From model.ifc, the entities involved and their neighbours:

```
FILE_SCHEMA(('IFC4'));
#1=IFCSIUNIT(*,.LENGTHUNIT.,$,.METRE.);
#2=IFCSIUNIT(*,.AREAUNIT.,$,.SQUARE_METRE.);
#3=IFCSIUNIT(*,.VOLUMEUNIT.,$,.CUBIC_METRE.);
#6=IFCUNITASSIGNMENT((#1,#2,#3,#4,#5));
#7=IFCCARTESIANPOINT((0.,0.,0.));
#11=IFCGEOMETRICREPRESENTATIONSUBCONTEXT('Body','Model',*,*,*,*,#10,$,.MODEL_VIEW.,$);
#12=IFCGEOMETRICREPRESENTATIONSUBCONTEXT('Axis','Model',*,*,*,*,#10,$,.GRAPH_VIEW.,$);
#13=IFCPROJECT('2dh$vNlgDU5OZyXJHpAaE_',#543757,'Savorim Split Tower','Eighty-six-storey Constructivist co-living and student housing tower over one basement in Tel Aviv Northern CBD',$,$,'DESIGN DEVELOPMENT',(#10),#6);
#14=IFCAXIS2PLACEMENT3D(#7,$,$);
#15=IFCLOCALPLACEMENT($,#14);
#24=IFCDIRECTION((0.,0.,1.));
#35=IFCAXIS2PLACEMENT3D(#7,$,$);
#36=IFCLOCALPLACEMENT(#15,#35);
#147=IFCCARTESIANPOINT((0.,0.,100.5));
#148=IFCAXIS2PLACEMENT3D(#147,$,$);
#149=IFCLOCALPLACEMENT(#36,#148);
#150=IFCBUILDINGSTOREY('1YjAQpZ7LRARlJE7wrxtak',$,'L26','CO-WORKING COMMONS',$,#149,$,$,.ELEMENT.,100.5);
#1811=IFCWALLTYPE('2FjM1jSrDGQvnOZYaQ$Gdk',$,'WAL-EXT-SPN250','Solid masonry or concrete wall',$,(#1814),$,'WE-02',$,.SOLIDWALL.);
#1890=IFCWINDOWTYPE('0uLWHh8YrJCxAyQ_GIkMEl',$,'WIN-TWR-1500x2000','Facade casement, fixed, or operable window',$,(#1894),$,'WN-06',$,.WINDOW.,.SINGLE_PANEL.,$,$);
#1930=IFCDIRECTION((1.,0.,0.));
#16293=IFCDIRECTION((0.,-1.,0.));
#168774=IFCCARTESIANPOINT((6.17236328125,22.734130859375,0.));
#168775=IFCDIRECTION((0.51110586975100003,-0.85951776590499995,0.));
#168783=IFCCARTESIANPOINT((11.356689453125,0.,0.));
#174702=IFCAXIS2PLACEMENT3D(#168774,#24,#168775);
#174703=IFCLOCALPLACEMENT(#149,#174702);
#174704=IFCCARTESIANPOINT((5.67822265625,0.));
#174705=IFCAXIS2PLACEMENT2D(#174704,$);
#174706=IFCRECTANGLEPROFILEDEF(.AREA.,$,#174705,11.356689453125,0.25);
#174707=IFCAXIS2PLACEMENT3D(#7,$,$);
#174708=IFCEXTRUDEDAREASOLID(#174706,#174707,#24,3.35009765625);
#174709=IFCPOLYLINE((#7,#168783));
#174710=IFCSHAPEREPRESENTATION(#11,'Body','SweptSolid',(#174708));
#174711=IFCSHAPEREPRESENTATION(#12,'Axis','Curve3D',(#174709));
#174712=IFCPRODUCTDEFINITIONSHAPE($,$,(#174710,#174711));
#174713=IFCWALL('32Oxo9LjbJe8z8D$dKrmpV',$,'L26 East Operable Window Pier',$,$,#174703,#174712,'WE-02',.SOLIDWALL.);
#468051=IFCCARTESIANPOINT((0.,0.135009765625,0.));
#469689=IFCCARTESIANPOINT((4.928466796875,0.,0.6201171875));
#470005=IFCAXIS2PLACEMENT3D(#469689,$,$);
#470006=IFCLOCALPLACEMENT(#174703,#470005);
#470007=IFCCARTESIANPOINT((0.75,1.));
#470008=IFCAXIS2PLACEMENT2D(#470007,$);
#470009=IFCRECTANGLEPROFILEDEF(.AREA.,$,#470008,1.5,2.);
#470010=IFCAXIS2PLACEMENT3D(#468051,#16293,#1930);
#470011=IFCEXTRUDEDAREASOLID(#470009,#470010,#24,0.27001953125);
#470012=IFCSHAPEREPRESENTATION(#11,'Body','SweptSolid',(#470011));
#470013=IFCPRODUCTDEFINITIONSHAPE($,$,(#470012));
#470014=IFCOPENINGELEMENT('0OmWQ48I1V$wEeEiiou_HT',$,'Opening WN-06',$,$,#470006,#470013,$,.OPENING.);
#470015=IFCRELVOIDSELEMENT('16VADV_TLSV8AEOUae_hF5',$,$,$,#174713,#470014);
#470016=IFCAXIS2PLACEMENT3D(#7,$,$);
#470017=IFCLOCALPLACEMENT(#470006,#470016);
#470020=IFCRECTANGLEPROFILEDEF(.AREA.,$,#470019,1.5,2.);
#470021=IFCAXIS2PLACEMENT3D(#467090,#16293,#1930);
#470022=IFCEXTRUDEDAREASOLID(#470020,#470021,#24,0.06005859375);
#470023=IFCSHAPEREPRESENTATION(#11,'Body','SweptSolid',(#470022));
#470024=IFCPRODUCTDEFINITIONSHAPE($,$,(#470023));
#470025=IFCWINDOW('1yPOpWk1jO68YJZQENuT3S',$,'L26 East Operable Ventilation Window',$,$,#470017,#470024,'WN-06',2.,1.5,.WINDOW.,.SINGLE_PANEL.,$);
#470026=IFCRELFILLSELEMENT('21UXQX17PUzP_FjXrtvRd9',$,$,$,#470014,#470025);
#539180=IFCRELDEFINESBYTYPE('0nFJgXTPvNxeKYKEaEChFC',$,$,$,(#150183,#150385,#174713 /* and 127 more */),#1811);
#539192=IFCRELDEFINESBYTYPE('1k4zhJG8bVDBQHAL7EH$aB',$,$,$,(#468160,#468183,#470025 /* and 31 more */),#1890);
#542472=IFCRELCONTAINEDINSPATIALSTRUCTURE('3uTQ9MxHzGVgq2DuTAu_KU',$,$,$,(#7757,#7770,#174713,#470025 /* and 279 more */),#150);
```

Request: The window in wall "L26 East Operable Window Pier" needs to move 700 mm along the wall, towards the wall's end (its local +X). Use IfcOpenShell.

```python
import ifcopenshell
import ifcopenshell.api.geometry
import ifcopenshell.util.placement

model = ifcopenshell.open("model.ifc")

window = model.by_guid("1yPOpWk1jO68YJZQENuT3S")
opening = window.FillsVoids[0].RelatingOpeningElement
wall = opening.VoidsElements[0].RelatingBuildingElement

wall_matrix = ifcopenshell.util.placement.get_local_placement(wall.ObjectPlacement)
shift = wall_matrix[:3, 0] * 0.7
before = ifcopenshell.util.placement.get_local_placement(window.ObjectPlacement)[:3, 3].copy()

# The window is placed relative to its opening, so it follows when the opening moves.
matrix = ifcopenshell.util.placement.get_local_placement(opening.ObjectPlacement)
matrix[:3, 3] += shift
ifcopenshell.api.geometry.edit_object_placement(
    model, product=opening, matrix=matrix, is_si=False, should_transform_children=True
)

after = ifcopenshell.util.placement.get_local_placement(window.ObjectPlacement)[:3, 3]
print("window moved by", (after - before).round(3) + 0.0)

model.write("model_v2.ifc")
```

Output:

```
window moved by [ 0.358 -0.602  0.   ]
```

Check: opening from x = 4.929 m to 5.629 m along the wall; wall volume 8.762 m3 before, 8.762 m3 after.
